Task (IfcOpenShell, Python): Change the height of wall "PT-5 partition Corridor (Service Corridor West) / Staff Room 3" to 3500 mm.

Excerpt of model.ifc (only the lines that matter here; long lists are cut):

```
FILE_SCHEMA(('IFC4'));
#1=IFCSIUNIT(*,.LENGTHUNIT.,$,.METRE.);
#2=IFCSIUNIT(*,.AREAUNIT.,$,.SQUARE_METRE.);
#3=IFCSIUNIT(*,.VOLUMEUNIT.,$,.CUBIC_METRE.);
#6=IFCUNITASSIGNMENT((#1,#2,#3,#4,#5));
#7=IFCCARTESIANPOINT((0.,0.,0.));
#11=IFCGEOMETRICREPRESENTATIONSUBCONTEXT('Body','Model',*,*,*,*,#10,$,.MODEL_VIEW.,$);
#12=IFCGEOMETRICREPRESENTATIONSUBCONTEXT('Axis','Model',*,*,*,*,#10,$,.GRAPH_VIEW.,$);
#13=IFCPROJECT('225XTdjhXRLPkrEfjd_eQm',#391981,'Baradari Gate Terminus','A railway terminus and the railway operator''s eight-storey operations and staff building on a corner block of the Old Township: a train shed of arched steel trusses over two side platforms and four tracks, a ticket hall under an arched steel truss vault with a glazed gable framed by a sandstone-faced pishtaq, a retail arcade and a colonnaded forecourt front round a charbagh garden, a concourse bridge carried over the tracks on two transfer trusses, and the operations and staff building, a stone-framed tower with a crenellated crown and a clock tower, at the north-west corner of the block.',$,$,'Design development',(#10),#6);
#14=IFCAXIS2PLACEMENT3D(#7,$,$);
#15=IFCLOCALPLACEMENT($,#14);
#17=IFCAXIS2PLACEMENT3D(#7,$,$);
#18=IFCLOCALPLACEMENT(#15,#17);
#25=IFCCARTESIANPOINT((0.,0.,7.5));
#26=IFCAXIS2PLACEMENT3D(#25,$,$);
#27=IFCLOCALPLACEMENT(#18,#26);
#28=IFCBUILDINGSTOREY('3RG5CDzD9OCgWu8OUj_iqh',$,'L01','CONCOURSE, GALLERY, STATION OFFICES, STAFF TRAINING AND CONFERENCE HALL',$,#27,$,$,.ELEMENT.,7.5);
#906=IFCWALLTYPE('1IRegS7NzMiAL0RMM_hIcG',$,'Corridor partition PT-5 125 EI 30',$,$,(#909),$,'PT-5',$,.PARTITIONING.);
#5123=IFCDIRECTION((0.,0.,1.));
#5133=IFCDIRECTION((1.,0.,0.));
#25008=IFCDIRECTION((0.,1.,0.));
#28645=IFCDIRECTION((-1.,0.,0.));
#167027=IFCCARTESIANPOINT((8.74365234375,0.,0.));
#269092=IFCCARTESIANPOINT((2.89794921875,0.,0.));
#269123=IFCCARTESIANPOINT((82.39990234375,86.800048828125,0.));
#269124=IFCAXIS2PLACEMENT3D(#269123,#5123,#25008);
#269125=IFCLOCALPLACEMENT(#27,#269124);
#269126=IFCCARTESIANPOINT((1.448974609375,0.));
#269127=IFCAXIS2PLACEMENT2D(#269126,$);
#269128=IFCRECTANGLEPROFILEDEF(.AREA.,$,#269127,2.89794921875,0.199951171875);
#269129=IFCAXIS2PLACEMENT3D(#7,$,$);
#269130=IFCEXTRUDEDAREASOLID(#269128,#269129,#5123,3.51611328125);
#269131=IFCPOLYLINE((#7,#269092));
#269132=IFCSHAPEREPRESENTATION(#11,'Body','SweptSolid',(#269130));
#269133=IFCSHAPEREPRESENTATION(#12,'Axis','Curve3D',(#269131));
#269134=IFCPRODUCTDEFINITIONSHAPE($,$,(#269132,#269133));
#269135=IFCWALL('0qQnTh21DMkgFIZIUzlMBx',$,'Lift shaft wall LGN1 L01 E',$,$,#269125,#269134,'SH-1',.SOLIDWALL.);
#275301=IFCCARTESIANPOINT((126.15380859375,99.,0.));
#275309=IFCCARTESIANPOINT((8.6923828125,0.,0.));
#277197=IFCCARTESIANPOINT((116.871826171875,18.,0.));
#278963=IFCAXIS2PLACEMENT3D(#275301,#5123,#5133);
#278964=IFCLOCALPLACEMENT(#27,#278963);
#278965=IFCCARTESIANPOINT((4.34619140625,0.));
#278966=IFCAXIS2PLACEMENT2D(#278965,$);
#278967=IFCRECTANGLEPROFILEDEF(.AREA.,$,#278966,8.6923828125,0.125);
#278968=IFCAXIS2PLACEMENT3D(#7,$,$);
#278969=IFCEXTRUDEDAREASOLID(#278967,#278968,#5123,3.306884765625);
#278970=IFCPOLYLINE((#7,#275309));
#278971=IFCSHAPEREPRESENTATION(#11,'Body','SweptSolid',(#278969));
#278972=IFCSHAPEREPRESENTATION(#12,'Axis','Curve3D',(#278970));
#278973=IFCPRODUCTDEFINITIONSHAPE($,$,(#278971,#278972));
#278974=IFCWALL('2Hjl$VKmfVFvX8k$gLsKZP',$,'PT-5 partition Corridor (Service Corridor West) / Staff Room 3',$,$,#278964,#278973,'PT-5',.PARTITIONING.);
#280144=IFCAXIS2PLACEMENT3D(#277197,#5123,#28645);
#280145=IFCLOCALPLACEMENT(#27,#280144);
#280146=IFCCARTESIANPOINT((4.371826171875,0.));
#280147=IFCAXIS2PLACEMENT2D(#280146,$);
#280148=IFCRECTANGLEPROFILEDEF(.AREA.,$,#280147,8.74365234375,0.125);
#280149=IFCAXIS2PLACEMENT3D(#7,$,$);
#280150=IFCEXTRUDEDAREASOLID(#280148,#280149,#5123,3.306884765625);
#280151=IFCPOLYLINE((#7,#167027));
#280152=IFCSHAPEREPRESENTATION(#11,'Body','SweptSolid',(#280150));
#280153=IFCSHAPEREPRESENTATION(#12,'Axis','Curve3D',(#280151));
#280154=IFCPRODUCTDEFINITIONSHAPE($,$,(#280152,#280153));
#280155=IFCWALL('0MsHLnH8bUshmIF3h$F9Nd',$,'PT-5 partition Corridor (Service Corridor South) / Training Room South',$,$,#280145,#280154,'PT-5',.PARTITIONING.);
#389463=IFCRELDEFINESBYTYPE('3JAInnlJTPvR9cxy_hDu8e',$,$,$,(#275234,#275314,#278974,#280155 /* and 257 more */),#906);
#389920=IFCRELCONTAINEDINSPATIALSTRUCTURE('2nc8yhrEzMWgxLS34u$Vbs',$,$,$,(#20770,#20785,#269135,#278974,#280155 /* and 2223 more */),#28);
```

```python
import ifcopenshell
import ifcopenshell.geom
import ifcopenshell.util.representation
import ifcopenshell.util.shape
import ifcopenshell.util.unit

model = ifcopenshell.open("model.ifc")
unit_scale = ifcopenshell.util.unit.calculate_unit_scale(model)
settings = ifcopenshell.geom.settings()


def volume(element):
    """Net volume in cubic metres, openings subtracted."""
    shape = ifcopenshell.geom.create_shape(settings, element)
    return ifcopenshell.util.shape.get_volume(shape.geometry)


wall = model.by_guid("2Hjl$VKmfVFvX8k$gLsKZP")
before = volume(wall)

body = ifcopenshell.util.representation.get_representation(wall, "Model", "Body")
solid = body.Items[0]
old_height = solid.Depth
solid.Depth = 3.5 / unit_scale
after = volume(wall)

print(f"height {old_height:g} -> {solid.Depth:g}, volume {before:.3f} -> {after:.3f} m3")

model.write("model_updated.ifc")
```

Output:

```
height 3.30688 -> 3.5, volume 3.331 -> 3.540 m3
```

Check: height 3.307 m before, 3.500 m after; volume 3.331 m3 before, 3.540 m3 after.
